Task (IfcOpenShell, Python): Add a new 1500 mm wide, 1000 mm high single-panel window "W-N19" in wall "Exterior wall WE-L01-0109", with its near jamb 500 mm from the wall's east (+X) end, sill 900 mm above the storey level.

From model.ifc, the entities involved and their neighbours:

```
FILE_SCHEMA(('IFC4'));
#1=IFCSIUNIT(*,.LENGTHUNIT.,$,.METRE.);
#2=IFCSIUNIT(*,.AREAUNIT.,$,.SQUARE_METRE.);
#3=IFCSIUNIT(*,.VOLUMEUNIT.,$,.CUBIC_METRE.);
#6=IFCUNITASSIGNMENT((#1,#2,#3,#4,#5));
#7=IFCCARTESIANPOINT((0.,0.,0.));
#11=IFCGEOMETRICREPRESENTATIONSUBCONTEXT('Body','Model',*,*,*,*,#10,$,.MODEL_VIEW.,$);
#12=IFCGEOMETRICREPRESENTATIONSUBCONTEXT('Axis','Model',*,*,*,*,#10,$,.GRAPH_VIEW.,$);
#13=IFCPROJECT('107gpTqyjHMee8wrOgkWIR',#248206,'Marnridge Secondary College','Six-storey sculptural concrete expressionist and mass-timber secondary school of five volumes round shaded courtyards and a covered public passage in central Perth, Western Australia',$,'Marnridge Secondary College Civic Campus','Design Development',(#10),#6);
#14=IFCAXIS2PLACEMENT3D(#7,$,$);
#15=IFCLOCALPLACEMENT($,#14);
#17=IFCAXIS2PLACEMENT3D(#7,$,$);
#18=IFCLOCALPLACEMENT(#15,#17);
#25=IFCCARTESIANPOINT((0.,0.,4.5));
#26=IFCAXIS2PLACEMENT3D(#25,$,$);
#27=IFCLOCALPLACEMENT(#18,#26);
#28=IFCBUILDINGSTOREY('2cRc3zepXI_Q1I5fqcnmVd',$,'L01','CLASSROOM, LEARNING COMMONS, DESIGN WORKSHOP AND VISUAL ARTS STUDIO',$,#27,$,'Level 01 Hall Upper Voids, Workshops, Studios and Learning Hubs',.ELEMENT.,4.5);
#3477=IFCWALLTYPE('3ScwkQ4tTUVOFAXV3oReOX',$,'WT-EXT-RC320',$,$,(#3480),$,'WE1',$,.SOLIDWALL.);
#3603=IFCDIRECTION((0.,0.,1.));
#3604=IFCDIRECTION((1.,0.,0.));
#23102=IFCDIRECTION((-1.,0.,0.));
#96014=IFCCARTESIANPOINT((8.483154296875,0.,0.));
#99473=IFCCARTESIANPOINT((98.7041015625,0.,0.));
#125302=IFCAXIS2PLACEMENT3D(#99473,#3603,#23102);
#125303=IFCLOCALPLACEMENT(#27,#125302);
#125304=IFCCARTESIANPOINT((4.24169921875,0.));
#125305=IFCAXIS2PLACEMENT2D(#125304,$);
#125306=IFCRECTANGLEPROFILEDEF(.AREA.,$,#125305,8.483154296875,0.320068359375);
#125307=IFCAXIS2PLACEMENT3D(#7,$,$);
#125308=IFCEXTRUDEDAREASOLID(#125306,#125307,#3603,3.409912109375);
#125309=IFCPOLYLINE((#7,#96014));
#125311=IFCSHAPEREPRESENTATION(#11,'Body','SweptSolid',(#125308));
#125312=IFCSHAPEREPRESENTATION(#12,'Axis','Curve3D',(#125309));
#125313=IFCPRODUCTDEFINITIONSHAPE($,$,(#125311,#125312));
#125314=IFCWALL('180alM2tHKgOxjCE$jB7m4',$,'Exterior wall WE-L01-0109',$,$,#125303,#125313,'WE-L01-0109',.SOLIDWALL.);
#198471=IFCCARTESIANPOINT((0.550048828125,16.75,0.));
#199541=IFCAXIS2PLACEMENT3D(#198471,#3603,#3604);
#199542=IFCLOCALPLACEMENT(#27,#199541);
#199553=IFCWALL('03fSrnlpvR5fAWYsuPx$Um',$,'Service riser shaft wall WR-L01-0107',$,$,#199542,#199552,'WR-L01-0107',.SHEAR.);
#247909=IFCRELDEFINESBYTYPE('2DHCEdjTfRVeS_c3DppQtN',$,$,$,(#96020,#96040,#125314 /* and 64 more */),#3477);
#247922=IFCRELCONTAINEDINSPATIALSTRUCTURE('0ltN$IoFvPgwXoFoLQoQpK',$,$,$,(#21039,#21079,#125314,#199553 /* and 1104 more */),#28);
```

```python
import numpy as np
import ifcopenshell
import ifcopenshell.api.feature
import ifcopenshell.api.geometry
import ifcopenshell.api.root
import ifcopenshell.api.spatial
import ifcopenshell.geom
import ifcopenshell.util.element
import ifcopenshell.util.placement
import ifcopenshell.util.representation
import ifcopenshell.util.shape
import ifcopenshell.util.unit

model = ifcopenshell.open("model.ifc")
unit_scale = ifcopenshell.util.unit.calculate_unit_scale(model)
settings = ifcopenshell.geom.settings()


def volume(element):
    """Net volume in cubic metres, openings subtracted."""
    shape = ifcopenshell.geom.create_shape(settings, element)
    return ifcopenshell.util.shape.get_volume(shape.geometry)


wall = model.by_guid("180alM2tHKgOxjCE$jB7m4")
storey = ifcopenshell.util.element.get_container(wall, ifc_class="IfcBuildingStorey")
context = ifcopenshell.util.representation.get_context(model, "Model", "Body", "MODEL_VIEW")
before = volume(wall)

width, height, from_end, sill = 1.5, 1, 0.5, 0.9  # metres

# The wall runs along its own X axis, and the end named is its -X end.
wall_shape = ifcopenshell.geom.create_shape(settings, wall)
x, y, z = ifcopenshell.util.shape.get_vertices(wall_shape.geometry).T
start = x.min() + from_end
face, thickness = float(y.min()), float(y.max() - y.min())
wall_matrix = ifcopenshell.util.placement.get_local_placement(wall.ObjectPlacement)
level = ifcopenshell.util.placement.get_local_placement(storey.ObjectPlacement)[2, 3]


def in_wall(x, y):
    """Placement at x, y metres in the wall's axes, at sill height."""
    matrix = wall_matrix.copy()
    matrix[:, 3] = wall_matrix @ np.array([x / unit_scale, y / unit_scale, 0.0, 1.0])
    matrix[2, 3] = level + sill / unit_scale
    return matrix


# Opening: a box that overshoots both wall faces by 50 mm.
opening = ifcopenshell.api.root.create_entity(model, ifc_class="IfcOpeningElement", predefined_type="OPENING")
box = ifcopenshell.api.geometry.add_wall_representation(
    model, context=context, length=width, height=height, thickness=thickness + 0.1
)
ifcopenshell.api.geometry.assign_representation(model, product=opening, representation=box)
ifcopenshell.api.geometry.edit_object_placement(model, product=opening, matrix=in_wall(start, face - 0.05), is_si=False)
ifcopenshell.api.feature.add_feature(model, feature=opening, element=wall)

window = ifcopenshell.api.root.create_entity(model, ifc_class="IfcWindow", name="W-N19", predefined_type="WINDOW")
window.OverallWidth, window.OverallHeight = width / unit_scale, height / unit_scale
window.PartitioningType = "SINGLE_PANEL"
body = ifcopenshell.api.geometry.add_window_representation(
    model,
    context=context,
    overall_width=window.OverallWidth,
    overall_height=window.OverallHeight,
    partition_type="SINGLE_PANEL",
)
ifcopenshell.api.geometry.assign_representation(model, product=window, representation=body)
ifcopenshell.api.spatial.assign_container(model, products=[window], relating_structure=storey)
ifcopenshell.api.feature.add_filling(model, opening=opening, element=window)

# Centre the window in the wall's thickness.
ifcopenshell.api.geometry.edit_object_placement(model, product=window, matrix=in_wall(start, face), is_si=False)
window_shape = ifcopenshell.geom.create_shape(settings, window)
depth = ifcopenshell.util.shape.get_vertices(window_shape.geometry)[:, 1]
offset = face + thickness / 2 - (depth.min() + depth.max()) / 2
ifcopenshell.api.geometry.edit_object_placement(model, product=window, matrix=in_wall(start, offset), is_si=False)

after = volume(wall)

print(f"wall volume {before:.3f} -> {after:.3f} m3")

model.write("model_v2.ifc")
```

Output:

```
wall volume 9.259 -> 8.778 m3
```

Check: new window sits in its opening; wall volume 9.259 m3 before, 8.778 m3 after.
